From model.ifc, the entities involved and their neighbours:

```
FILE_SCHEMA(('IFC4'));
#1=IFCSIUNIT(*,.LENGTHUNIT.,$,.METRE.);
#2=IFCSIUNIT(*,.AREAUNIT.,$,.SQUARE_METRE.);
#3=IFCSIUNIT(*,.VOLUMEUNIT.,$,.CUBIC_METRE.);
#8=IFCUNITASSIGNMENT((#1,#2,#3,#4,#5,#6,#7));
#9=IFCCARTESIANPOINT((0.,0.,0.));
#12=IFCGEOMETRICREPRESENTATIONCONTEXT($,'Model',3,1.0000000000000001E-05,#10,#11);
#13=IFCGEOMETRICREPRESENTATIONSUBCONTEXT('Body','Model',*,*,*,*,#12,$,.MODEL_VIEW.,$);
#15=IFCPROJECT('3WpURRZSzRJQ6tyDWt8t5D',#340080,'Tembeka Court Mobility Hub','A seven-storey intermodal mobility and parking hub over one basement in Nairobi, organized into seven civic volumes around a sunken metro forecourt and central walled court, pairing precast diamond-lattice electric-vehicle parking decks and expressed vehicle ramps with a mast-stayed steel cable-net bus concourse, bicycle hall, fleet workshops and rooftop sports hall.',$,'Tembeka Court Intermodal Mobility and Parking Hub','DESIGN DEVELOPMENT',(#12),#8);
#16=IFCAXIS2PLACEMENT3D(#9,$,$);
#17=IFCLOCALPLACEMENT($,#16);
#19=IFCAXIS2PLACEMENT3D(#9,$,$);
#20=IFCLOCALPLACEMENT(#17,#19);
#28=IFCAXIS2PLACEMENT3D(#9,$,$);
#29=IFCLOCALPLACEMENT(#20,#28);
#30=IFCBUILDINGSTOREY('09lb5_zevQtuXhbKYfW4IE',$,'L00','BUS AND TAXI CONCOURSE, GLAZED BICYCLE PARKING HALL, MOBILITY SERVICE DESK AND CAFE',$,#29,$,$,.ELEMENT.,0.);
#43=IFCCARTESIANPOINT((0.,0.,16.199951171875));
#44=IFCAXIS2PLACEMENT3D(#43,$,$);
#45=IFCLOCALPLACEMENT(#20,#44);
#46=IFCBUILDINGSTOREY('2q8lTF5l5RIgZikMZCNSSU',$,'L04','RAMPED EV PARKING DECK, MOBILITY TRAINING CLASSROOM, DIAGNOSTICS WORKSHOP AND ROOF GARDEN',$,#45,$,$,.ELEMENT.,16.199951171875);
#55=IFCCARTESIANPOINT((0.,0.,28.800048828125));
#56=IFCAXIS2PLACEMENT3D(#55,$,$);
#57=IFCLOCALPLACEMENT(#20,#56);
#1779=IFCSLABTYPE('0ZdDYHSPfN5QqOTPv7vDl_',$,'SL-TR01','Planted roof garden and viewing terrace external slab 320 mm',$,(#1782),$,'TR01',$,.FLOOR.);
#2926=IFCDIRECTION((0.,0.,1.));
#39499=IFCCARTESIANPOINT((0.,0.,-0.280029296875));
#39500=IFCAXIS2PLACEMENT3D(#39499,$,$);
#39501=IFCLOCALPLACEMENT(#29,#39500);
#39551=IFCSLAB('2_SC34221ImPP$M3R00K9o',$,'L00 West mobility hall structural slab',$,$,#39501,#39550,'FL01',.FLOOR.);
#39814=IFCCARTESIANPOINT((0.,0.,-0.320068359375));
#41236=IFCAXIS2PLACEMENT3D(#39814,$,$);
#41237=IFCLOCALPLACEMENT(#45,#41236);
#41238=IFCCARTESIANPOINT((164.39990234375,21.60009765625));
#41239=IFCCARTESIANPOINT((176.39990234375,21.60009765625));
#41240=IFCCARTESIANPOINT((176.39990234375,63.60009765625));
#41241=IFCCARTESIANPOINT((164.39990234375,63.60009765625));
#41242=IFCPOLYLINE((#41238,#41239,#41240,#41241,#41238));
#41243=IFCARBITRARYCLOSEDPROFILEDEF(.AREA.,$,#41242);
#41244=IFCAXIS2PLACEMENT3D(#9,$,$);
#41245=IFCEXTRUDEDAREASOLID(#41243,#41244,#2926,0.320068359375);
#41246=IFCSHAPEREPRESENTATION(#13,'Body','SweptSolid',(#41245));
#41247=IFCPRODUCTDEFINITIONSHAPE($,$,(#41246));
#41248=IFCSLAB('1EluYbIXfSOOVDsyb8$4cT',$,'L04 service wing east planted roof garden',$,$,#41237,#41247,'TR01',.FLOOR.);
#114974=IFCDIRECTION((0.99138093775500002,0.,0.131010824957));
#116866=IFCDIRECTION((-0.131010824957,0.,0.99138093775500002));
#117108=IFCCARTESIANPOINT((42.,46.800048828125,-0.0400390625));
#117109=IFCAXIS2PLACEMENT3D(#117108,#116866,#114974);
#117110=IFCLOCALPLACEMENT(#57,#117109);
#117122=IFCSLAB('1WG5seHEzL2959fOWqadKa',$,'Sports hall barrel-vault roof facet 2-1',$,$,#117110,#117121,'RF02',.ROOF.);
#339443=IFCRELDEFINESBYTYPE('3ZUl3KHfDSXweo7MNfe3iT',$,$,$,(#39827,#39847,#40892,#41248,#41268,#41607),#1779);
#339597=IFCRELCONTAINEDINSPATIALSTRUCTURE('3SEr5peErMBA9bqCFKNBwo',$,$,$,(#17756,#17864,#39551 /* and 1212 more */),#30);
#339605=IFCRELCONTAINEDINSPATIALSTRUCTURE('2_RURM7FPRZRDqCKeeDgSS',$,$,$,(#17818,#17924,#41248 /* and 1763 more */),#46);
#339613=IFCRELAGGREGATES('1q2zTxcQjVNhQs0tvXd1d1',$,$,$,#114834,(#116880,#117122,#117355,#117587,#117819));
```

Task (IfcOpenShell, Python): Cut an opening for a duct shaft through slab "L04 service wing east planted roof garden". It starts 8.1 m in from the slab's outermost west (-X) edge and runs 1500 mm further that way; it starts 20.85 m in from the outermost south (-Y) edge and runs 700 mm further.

```python
import numpy as np
import ifcopenshell
import ifcopenshell.api.feature
import ifcopenshell.api.geometry
import ifcopenshell.api.root
import ifcopenshell.geom
import ifcopenshell.util.placement
import ifcopenshell.util.representation
import ifcopenshell.util.shape
import ifcopenshell.util.unit

model = ifcopenshell.open("model.ifc")
unit_scale = ifcopenshell.util.unit.calculate_unit_scale(model)
settings = ifcopenshell.geom.settings()


def volume(element):
    """Net volume in cubic metres, openings subtracted."""
    shape = ifcopenshell.geom.create_shape(settings, element)
    return ifcopenshell.util.shape.get_volume(shape.geometry)


slab = model.by_id(41248)
before = volume(slab)

# Extent in the slab's own axes, in metres. The edges named are its -X and -Y sides.
slab_shape = ifcopenshell.geom.create_shape(settings, slab)
vertices = ifcopenshell.util.shape.get_vertices(slab_shape.geometry)
x_min, y_min, bottom = vertices.min(axis=0)
top = vertices[:, 2].max()

opening = ifcopenshell.api.root.create_entity(model, ifc_class="IfcOpeningElement", name="Duct shaft opening", predefined_type="OPENING")
context = ifcopenshell.util.representation.get_context(model, "Model", "Body", "MODEL_VIEW")
width, depth = 1.5, 0.7
outline = [(0.0, 0.0), (width, 0.0), (width, depth), (0.0, depth), (0.0, 0.0)]
# Overshoot both faces by 50 mm so the cut is clean.
shape = ifcopenshell.api.geometry.add_slab_representation(
    model, context=context, depth=top - bottom + 0.1, polyline=outline
)
ifcopenshell.api.geometry.assign_representation(model, product=opening, representation=shape)

matrix = ifcopenshell.util.placement.get_local_placement(slab.ObjectPlacement)
matrix[:, 3] = matrix @ np.append(np.array([x_min + 8.1, y_min + 20.85, bottom - 0.05]) / unit_scale, 1.0)
ifcopenshell.api.geometry.edit_object_placement(model, product=opening, matrix=matrix, is_si=False)
ifcopenshell.api.feature.add_feature(model, feature=opening, element=slab)

after = volume(slab)

print(f"slab volume {before:.3f} -> {after:.3f} m3")

model.write("model_updated.ifc")
```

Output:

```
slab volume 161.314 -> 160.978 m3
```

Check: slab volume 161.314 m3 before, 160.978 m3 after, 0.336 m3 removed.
